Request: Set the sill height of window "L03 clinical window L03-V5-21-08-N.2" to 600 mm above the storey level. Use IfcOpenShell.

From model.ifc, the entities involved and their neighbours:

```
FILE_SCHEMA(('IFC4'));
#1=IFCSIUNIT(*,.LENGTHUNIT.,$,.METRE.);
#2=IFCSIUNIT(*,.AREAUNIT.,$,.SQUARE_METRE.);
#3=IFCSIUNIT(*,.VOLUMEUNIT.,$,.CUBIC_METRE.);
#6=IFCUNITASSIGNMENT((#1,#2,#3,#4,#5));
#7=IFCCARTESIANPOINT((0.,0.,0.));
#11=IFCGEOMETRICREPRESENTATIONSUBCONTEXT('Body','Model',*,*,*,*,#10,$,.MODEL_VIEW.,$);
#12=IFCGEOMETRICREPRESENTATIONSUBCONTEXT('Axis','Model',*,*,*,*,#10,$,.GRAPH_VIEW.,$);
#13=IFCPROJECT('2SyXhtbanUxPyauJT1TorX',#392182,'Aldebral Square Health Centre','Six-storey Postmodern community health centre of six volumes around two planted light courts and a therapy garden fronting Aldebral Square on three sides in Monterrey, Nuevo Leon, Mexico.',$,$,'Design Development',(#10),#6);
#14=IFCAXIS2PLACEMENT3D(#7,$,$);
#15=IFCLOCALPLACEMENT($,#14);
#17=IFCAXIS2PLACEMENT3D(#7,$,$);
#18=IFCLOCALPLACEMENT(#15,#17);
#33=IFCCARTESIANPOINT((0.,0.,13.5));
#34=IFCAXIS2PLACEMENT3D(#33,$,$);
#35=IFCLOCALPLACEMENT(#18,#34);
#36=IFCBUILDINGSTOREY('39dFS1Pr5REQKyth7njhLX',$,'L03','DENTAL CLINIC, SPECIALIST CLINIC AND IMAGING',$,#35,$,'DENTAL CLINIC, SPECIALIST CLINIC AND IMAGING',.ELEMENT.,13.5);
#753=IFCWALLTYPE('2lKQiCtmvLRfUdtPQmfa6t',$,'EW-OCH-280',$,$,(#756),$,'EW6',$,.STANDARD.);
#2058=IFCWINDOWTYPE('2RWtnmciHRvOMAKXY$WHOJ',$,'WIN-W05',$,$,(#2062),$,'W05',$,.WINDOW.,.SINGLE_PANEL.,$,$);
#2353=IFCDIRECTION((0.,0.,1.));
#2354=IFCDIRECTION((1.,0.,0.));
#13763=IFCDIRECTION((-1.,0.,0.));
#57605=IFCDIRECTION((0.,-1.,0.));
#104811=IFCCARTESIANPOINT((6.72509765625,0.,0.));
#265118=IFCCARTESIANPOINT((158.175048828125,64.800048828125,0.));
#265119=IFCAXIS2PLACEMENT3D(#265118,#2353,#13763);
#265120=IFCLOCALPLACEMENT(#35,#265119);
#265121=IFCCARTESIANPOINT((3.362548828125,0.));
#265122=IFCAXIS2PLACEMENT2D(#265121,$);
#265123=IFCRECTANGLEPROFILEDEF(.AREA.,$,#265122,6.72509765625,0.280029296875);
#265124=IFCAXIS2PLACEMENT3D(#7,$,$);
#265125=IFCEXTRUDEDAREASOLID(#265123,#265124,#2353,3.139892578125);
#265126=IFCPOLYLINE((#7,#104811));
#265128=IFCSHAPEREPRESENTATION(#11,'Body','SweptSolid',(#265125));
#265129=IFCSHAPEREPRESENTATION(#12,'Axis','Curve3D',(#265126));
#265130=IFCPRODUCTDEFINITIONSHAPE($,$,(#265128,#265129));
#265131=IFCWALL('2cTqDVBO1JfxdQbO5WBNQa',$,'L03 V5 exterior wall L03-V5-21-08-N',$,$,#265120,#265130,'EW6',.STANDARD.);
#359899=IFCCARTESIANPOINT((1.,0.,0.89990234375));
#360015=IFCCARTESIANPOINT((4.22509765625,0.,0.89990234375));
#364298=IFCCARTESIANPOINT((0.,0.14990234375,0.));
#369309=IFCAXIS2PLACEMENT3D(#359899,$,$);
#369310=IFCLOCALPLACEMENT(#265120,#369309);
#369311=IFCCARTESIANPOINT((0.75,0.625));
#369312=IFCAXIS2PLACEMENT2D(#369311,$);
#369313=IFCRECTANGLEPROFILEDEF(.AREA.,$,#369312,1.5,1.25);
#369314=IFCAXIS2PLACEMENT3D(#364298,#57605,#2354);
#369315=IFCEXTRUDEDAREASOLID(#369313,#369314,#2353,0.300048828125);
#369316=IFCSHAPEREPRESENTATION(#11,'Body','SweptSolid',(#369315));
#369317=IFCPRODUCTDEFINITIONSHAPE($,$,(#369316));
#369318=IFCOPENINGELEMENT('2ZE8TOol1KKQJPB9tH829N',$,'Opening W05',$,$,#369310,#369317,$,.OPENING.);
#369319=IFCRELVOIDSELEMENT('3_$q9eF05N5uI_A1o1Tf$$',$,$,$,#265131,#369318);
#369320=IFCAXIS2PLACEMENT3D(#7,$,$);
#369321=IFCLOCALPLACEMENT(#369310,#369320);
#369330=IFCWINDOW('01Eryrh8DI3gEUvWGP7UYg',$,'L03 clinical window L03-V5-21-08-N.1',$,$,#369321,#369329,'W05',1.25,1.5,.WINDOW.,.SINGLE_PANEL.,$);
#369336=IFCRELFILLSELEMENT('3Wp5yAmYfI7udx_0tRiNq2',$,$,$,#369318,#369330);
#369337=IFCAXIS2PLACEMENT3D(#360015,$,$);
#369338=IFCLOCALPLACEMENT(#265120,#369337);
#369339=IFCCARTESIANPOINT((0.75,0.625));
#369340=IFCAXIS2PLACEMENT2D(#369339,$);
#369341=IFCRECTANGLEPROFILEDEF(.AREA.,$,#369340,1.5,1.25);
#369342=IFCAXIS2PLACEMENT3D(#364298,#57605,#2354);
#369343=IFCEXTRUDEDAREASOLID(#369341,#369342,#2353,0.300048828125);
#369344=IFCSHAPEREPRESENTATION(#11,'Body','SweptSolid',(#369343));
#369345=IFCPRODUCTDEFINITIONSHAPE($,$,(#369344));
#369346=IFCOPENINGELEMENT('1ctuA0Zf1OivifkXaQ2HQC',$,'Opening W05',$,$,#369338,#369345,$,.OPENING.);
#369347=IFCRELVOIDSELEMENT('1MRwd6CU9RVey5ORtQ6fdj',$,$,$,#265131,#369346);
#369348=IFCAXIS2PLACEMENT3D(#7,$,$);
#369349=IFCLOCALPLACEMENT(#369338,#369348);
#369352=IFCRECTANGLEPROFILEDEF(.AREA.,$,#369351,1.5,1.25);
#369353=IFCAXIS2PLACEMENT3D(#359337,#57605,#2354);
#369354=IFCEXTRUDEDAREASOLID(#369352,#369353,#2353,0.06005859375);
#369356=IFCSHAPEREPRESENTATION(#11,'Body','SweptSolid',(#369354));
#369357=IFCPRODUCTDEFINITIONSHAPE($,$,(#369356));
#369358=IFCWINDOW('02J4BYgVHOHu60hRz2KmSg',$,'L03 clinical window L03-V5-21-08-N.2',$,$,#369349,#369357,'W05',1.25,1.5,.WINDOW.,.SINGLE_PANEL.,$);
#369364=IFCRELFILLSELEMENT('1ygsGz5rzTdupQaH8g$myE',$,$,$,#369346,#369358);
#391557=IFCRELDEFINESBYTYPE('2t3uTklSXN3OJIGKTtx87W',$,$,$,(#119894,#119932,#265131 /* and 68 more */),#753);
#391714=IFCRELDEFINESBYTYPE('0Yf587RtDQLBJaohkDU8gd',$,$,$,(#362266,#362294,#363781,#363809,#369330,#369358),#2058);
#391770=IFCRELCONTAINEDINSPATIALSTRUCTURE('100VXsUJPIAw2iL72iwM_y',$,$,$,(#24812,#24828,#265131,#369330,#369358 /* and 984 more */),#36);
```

```python
import numpy as np
import ifcopenshell
import ifcopenshell.api.geometry
import ifcopenshell.geom
import ifcopenshell.util.element
import ifcopenshell.util.placement
import ifcopenshell.util.shape
import ifcopenshell.util.unit

model = ifcopenshell.open("model.ifc")
unit_scale = ifcopenshell.util.unit.calculate_unit_scale(model)

window = model.by_guid("02J4BYgVHOHu60hRz2KmSg")
opening = window.FillsVoids[0].RelatingOpeningElement
storey = ifcopenshell.util.element.get_container(window, ifc_class="IfcBuildingStorey")
level = ifcopenshell.util.placement.get_local_placement(storey.ObjectPlacement)[2, 3]

# The opening's origin need not be at the sill, so measure its lowest point.
shape = ifcopenshell.geom.create_shape(ifcopenshell.geom.settings(), opening)
bottom = ifcopenshell.util.shape.get_shape_bottom_elevation(shape, shape.geometry) / unit_scale
dz = level + 0.6 - bottom

shift = np.array([0.0, 0.0, dz])
# The window is placed relative to its opening, so it follows when the opening moves.
matrix = ifcopenshell.util.placement.get_local_placement(opening.ObjectPlacement)
matrix[:3, 3] += shift
ifcopenshell.api.geometry.edit_object_placement(
    model, product=opening, matrix=matrix, is_si=False, should_transform_children=True
)

print(f"moved by {dz * unit_scale:+.3f} m")

model.write("model_updated.ifc")
```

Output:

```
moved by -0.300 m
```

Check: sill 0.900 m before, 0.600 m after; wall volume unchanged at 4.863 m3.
